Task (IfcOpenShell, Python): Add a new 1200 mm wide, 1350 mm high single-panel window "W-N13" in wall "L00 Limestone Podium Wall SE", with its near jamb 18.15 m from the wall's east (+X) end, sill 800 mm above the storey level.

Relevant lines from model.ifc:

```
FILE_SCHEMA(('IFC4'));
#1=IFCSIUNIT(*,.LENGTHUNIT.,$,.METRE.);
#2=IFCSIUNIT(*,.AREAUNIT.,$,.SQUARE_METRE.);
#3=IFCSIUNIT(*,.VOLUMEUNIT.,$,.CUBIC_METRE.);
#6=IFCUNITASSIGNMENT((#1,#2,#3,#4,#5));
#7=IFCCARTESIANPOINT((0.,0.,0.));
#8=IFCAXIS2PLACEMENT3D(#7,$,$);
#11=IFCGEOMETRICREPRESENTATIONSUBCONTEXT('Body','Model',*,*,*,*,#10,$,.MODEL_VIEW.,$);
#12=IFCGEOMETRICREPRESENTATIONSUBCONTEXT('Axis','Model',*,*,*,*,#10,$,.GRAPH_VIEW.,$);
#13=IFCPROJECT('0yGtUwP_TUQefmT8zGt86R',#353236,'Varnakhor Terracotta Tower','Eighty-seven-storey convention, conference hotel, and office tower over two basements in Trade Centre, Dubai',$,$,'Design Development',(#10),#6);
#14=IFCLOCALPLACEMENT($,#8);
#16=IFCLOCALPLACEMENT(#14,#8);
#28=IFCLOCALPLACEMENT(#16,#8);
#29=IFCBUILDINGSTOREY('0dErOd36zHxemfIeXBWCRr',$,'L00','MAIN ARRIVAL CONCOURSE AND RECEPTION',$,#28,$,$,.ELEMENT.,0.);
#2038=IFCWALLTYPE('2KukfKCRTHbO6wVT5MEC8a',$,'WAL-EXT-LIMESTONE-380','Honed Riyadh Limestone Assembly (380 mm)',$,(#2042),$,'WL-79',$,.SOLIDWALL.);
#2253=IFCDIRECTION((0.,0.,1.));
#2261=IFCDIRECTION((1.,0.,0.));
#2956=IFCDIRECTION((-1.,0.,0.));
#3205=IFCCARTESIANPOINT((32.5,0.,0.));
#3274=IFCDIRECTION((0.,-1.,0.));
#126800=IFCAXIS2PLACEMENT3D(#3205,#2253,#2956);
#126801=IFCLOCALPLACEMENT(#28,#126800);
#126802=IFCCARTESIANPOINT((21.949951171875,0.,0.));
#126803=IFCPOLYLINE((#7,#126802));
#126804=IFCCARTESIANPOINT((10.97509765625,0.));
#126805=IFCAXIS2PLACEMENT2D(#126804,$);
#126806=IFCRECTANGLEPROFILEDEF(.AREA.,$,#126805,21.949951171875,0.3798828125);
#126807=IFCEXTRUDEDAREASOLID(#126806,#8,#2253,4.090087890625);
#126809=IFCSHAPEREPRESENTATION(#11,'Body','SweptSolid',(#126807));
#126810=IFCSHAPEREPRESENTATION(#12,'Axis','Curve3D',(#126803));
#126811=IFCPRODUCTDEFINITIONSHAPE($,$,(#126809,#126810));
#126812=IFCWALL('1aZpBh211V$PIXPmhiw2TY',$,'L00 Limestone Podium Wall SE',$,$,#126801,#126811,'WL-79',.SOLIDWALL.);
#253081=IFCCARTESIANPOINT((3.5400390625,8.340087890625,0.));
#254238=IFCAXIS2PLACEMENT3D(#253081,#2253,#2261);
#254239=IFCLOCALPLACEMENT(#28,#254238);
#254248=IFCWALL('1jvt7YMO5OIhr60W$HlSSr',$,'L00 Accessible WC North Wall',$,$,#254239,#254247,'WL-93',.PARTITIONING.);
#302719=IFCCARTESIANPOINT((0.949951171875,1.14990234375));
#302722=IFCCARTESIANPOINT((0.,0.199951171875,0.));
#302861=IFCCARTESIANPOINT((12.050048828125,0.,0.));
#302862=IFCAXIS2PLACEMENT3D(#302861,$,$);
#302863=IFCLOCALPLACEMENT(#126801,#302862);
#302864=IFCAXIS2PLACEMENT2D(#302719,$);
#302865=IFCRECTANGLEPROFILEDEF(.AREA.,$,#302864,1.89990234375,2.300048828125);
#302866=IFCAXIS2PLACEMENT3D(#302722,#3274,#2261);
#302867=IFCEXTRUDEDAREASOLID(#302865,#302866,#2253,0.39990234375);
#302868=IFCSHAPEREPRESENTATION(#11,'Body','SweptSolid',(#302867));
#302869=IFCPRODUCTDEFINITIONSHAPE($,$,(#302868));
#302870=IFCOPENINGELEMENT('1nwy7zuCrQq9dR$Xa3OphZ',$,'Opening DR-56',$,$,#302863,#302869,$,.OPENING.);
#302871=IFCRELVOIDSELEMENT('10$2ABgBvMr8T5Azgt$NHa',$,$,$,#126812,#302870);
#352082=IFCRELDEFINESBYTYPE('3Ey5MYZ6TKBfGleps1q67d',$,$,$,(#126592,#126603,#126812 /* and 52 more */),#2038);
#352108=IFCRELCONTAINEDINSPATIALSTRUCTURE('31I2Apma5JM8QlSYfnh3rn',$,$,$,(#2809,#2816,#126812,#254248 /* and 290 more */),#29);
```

```python
import numpy as np
import ifcopenshell
import ifcopenshell.api.feature
import ifcopenshell.api.geometry
import ifcopenshell.api.root
import ifcopenshell.api.spatial
import ifcopenshell.geom
import ifcopenshell.util.element
import ifcopenshell.util.placement
import ifcopenshell.util.representation
import ifcopenshell.util.shape
import ifcopenshell.util.unit

model = ifcopenshell.open("model.ifc")
unit_scale = ifcopenshell.util.unit.calculate_unit_scale(model)
settings = ifcopenshell.geom.settings()


def volume(element):
    """Net volume in cubic metres, openings subtracted."""
    shape = ifcopenshell.geom.create_shape(settings, element)
    return ifcopenshell.util.shape.get_volume(shape.geometry)


wall = model.by_guid("1aZpBh211V$PIXPmhiw2TY")
storey = ifcopenshell.util.element.get_container(wall, ifc_class="IfcBuildingStorey")
context = ifcopenshell.util.representation.get_context(model, "Model", "Body", "MODEL_VIEW")
before = volume(wall)

width, height, from_end, sill = 1.2, 1.35, 18.15, 0.8  # metres

# The wall runs along its own X axis, and the end named is its -X end.
wall_shape = ifcopenshell.geom.create_shape(settings, wall)
x, y, z = ifcopenshell.util.shape.get_vertices(wall_shape.geometry).T
start = x.min() + from_end
face, thickness = float(y.min()), float(y.max() - y.min())
wall_matrix = ifcopenshell.util.placement.get_local_placement(wall.ObjectPlacement)
level = ifcopenshell.util.placement.get_local_placement(storey.ObjectPlacement)[2, 3]


def in_wall(x, y):
    """Placement at x, y metres in the wall's axes, at sill height."""
    matrix = wall_matrix.copy()
    matrix[:, 3] = wall_matrix @ np.array([x / unit_scale, y / unit_scale, 0.0, 1.0])
    matrix[2, 3] = level + sill / unit_scale
    return matrix


# Opening: a box that overshoots both wall faces by 50 mm.
opening = ifcopenshell.api.root.create_entity(model, ifc_class="IfcOpeningElement", predefined_type="OPENING")
box = ifcopenshell.api.geometry.add_wall_representation(
    model, context=context, length=width, height=height, thickness=thickness + 0.1
)
ifcopenshell.api.geometry.assign_representation(model, product=opening, representation=box)
ifcopenshell.api.geometry.edit_object_placement(model, product=opening, matrix=in_wall(start, face - 0.05), is_si=False)
ifcopenshell.api.feature.add_feature(model, feature=opening, element=wall)

window = ifcopenshell.api.root.create_entity(model, ifc_class="IfcWindow", name="W-N13", predefined_type="WINDOW")
window.OverallWidth, window.OverallHeight = width / unit_scale, height / unit_scale
window.PartitioningType = "SINGLE_PANEL"
body = ifcopenshell.api.geometry.add_window_representation(
    model,
    context=context,
    overall_width=window.OverallWidth,
    overall_height=window.OverallHeight,
    partition_type="SINGLE_PANEL",
)
ifcopenshell.api.geometry.assign_representation(model, product=window, representation=body)
ifcopenshell.api.spatial.assign_container(model, products=[window], relating_structure=storey)
ifcopenshell.api.feature.add_filling(model, opening=opening, element=window)

# Centre the window in the wall's thickness.
ifcopenshell.api.geometry.edit_object_placement(model, product=window, matrix=in_wall(start, face), is_si=False)
window_shape = ifcopenshell.geom.create_shape(settings, window)
depth = ifcopenshell.util.shape.get_vertices(window_shape.geometry)[:, 1]
offset = face + thickness / 2 - (depth.min() + depth.max()) / 2
ifcopenshell.api.geometry.edit_object_placement(model, product=window, matrix=in_wall(start, offset), is_si=False)

after = volume(wall)

print(f"wall volume {before:.3f} -> {after:.3f} m3")

model.write("model-out.ifc")
```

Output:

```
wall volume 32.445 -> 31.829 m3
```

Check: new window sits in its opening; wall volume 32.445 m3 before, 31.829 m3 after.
